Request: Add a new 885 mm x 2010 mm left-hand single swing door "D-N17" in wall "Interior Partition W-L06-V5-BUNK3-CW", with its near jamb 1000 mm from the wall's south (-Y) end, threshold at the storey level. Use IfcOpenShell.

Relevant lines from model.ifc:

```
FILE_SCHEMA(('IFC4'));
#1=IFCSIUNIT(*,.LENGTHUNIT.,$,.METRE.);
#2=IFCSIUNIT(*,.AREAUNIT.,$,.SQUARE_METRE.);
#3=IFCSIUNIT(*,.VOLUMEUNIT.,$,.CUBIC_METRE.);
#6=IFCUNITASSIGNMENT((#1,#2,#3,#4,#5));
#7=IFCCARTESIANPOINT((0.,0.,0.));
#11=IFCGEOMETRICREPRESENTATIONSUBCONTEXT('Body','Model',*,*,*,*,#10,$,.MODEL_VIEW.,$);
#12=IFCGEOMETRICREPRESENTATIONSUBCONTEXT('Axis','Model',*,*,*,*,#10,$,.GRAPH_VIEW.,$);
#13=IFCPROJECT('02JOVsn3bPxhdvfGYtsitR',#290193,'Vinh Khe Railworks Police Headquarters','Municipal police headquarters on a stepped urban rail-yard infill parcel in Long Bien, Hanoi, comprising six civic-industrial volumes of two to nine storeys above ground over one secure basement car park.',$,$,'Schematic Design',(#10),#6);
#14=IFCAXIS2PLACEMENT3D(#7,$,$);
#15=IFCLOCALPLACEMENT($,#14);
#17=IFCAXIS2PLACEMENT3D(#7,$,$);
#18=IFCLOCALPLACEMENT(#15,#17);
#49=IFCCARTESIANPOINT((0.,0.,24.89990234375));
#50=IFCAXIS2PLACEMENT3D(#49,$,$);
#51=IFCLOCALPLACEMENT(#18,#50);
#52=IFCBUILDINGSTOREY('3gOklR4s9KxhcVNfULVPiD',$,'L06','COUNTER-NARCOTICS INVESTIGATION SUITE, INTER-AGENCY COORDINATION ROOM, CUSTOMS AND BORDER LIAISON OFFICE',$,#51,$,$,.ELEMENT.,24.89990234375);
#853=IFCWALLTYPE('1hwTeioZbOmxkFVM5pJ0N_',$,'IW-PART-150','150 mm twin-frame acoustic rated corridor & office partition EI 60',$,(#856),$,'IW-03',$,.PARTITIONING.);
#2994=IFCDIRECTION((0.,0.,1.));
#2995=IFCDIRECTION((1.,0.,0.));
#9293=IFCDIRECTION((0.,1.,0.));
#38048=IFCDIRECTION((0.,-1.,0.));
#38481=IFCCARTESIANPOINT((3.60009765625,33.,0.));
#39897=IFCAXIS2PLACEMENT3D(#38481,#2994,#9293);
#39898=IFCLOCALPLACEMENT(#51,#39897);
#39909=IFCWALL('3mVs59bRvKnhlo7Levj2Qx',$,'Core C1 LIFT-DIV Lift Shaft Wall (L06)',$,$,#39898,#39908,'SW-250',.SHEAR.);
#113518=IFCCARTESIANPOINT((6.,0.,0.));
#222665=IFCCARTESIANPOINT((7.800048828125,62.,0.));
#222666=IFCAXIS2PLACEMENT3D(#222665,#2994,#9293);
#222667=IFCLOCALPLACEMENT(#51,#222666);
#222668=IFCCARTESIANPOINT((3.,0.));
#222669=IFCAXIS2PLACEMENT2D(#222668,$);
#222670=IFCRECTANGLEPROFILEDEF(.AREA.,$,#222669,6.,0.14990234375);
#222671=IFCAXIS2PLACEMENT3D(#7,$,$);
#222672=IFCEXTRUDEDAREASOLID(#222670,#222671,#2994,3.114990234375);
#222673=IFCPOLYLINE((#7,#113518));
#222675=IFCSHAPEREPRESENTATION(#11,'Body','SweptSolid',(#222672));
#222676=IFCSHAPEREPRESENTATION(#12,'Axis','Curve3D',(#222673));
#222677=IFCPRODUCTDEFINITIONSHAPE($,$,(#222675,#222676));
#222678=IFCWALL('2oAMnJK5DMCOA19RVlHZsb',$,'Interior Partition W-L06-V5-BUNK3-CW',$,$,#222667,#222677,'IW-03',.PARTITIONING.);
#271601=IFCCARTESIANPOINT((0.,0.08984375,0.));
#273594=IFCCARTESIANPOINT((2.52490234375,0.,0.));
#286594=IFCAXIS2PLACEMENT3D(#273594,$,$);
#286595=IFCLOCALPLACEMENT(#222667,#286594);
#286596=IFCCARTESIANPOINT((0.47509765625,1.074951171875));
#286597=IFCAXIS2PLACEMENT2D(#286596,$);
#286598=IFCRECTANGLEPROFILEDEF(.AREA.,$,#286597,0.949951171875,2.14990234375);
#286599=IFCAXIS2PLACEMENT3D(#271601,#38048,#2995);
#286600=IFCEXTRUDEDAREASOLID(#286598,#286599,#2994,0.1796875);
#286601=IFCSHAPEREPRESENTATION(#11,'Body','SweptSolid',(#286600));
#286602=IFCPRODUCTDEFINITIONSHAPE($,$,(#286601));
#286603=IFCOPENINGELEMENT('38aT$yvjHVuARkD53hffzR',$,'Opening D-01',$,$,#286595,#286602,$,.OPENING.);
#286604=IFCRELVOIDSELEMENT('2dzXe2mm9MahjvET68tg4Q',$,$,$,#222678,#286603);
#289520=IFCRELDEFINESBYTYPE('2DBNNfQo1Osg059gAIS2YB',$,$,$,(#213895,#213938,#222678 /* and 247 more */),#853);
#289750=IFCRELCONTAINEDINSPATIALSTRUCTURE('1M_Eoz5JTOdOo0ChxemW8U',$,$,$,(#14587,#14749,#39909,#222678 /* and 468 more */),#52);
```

```python
import numpy as np
import ifcopenshell
import ifcopenshell.api.feature
import ifcopenshell.api.geometry
import ifcopenshell.api.root
import ifcopenshell.api.spatial
import ifcopenshell.geom
import ifcopenshell.util.element
import ifcopenshell.util.placement
import ifcopenshell.util.representation
import ifcopenshell.util.shape
import ifcopenshell.util.unit

model = ifcopenshell.open("model.ifc")
unit_scale = ifcopenshell.util.unit.calculate_unit_scale(model)
settings = ifcopenshell.geom.settings()


def volume(element):
    """Net volume in cubic metres, openings subtracted."""
    shape = ifcopenshell.geom.create_shape(settings, element)
    return ifcopenshell.util.shape.get_volume(shape.geometry)


wall = model.by_guid("2oAMnJK5DMCOA19RVlHZsb")
storey = ifcopenshell.util.element.get_container(wall, ifc_class="IfcBuildingStorey")
context = ifcopenshell.util.representation.get_context(model, "Model", "Body", "MODEL_VIEW")
before = volume(wall)

width, height, from_end, sill = 0.885, 2.01, 1, 0.0  # metres

# The wall runs along its own X axis, and the end named is its -X end.
wall_shape = ifcopenshell.geom.create_shape(settings, wall)
x, y, z = ifcopenshell.util.shape.get_vertices(wall_shape.geometry).T
start = x.min() + from_end
face, thickness = float(y.min()), float(y.max() - y.min())
wall_matrix = ifcopenshell.util.placement.get_local_placement(wall.ObjectPlacement)
level = ifcopenshell.util.placement.get_local_placement(storey.ObjectPlacement)[2, 3]


def in_wall(x, y):
    """Placement at x, y metres in the wall's axes, at sill height."""
    matrix = wall_matrix.copy()
    matrix[:, 3] = wall_matrix @ np.array([x / unit_scale, y / unit_scale, 0.0, 1.0])
    matrix[2, 3] = level + sill / unit_scale
    return matrix


# Opening: a box that overshoots both wall faces by 50 mm.
opening = ifcopenshell.api.root.create_entity(model, ifc_class="IfcOpeningElement", predefined_type="OPENING")
box = ifcopenshell.api.geometry.add_wall_representation(
    model, context=context, length=width, height=height, thickness=thickness + 0.1
)
ifcopenshell.api.geometry.assign_representation(model, product=opening, representation=box)
ifcopenshell.api.geometry.edit_object_placement(model, product=opening, matrix=in_wall(start, face - 0.05), is_si=False)
ifcopenshell.api.feature.add_feature(model, feature=opening, element=wall)

door = ifcopenshell.api.root.create_entity(model, ifc_class="IfcDoor", name="D-N17", predefined_type="DOOR")
door.OverallWidth, door.OverallHeight = width / unit_scale, height / unit_scale
door.OperationType = "SINGLE_SWING_LEFT"
body = ifcopenshell.api.geometry.add_door_representation(
    model,
    context=context,
    overall_width=door.OverallWidth,
    overall_height=door.OverallHeight,
    operation_type="SINGLE_SWING_LEFT",
    lining_properties={"LiningDepth": thickness / unit_scale, "ThresholdDepth": thickness / unit_scale},
)
ifcopenshell.api.geometry.assign_representation(model, product=door, representation=body)
ifcopenshell.api.spatial.assign_container(model, products=[door], relating_structure=storey)
ifcopenshell.api.feature.add_filling(model, opening=opening, element=door)

# The lining spans the wall, so the door starts at the wall face.
ifcopenshell.api.geometry.edit_object_placement(model, product=door, matrix=in_wall(start, face), is_si=False)

after = volume(wall)

print(f"wall volume {before:.3f} -> {after:.3f} m3")

model.write("model_v2.ifc")
```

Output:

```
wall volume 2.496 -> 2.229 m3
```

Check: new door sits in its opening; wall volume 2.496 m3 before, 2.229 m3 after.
